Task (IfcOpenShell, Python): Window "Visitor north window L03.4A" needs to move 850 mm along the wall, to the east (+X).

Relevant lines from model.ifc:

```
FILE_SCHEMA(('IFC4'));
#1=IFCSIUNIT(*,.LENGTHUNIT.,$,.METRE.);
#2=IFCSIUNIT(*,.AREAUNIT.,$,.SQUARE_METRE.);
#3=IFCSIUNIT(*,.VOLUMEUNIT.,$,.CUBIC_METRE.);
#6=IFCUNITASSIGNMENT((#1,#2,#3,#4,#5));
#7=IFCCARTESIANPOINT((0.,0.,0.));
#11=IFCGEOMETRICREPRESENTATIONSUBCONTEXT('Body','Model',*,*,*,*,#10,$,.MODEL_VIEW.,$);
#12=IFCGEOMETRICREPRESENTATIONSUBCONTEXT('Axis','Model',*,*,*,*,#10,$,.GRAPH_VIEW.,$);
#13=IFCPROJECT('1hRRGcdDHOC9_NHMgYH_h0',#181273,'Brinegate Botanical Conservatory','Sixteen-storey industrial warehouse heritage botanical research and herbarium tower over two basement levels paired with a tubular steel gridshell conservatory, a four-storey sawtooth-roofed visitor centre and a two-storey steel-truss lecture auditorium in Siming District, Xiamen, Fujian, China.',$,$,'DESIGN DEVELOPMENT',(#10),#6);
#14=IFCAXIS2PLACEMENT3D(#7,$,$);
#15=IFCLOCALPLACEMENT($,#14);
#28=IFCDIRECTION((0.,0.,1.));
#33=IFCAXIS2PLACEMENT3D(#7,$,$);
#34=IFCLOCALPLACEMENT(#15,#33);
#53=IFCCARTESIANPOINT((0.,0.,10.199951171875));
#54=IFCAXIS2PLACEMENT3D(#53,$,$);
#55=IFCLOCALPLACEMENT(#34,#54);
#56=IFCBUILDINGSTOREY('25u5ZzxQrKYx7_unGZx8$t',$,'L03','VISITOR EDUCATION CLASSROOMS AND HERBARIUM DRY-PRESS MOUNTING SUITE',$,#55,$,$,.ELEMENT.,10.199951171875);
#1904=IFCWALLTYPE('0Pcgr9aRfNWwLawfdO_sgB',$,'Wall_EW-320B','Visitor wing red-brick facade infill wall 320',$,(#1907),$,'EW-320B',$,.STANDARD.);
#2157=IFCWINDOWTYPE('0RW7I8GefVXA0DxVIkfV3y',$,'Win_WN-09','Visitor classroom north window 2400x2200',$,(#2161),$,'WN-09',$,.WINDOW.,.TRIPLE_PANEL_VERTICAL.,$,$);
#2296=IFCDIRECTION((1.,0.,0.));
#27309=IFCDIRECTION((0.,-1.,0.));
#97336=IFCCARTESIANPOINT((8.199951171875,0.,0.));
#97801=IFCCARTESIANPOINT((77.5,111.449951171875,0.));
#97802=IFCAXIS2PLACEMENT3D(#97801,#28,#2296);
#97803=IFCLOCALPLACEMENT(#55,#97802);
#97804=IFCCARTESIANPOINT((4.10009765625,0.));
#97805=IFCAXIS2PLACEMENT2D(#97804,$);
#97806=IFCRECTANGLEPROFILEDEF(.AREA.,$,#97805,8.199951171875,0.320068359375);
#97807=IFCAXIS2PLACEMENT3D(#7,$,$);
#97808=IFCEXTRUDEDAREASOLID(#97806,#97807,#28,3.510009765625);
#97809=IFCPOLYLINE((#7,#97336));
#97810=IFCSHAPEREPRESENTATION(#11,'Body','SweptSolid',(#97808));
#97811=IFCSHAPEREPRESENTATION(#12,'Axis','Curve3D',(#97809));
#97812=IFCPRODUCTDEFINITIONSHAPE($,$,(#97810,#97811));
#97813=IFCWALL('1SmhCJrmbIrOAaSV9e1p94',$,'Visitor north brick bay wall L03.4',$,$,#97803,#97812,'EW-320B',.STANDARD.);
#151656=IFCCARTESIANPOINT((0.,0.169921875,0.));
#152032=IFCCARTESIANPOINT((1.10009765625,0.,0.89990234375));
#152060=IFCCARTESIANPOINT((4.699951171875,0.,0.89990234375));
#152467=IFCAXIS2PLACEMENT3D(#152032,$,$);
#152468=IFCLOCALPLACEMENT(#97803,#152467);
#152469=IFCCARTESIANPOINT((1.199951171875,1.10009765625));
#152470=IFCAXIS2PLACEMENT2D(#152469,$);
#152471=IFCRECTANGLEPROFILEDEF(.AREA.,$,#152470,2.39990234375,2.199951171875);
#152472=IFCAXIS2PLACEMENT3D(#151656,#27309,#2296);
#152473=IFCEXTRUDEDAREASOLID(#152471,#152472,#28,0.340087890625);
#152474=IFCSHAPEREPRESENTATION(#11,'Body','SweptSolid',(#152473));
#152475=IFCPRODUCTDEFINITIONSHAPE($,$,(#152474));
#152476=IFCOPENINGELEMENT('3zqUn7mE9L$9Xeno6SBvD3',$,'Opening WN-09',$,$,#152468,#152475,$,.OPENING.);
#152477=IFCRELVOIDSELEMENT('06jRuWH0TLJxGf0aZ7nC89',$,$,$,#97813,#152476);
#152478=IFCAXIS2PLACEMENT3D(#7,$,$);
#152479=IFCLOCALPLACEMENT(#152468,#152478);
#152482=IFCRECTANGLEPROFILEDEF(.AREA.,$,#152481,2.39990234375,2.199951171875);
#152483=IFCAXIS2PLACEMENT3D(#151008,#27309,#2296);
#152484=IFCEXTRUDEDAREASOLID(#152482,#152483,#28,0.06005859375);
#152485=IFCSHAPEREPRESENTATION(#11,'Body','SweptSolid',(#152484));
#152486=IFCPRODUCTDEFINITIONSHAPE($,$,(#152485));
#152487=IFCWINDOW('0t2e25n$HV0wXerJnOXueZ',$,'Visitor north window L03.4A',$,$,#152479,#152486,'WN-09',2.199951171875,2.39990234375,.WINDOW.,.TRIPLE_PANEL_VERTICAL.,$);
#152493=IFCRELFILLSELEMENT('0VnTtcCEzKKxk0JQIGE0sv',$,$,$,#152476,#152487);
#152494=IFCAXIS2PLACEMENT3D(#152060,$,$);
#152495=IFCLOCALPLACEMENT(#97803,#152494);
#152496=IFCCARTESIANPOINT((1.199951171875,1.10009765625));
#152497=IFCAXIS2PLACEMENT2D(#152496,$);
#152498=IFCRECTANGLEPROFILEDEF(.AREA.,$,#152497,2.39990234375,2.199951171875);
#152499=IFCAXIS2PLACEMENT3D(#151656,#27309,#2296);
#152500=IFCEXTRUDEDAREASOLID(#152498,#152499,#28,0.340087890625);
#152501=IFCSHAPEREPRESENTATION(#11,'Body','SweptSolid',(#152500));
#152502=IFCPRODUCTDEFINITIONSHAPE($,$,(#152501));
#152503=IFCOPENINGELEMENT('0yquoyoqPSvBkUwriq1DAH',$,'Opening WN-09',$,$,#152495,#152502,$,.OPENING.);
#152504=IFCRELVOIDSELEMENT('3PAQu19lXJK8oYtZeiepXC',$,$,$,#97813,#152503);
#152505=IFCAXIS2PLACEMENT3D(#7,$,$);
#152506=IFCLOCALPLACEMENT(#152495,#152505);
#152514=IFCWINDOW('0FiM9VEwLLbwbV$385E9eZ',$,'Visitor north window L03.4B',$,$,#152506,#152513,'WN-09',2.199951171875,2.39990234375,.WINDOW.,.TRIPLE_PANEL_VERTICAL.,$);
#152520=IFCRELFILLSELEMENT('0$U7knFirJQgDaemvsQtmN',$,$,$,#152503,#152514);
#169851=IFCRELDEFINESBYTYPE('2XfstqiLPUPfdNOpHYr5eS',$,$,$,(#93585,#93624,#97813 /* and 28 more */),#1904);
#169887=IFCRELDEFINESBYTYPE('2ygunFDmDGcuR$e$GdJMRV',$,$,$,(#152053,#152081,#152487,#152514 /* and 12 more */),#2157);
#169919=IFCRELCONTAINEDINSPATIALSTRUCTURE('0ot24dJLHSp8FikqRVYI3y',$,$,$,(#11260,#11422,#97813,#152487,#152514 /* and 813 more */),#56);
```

```python
import ifcopenshell
import ifcopenshell.api.geometry
import ifcopenshell.util.placement
import ifcopenshell.util.unit

model = ifcopenshell.open("model.ifc")
unit_scale = ifcopenshell.util.unit.calculate_unit_scale(model)

window = model.by_guid("0t2e25n$HV0wXerJnOXueZ")
opening = window.FillsVoids[0].RelatingOpeningElement
wall = opening.VoidsElements[0].RelatingBuildingElement

wall_matrix = ifcopenshell.util.placement.get_local_placement(wall.ObjectPlacement)
shift = wall_matrix[:3, 0] * 0.85 / unit_scale
before = ifcopenshell.util.placement.get_local_placement(window.ObjectPlacement)[:3, 3].copy()

# The window is placed relative to its opening, so it follows when the opening moves.
matrix = ifcopenshell.util.placement.get_local_placement(opening.ObjectPlacement)
matrix[:3, 3] += shift
ifcopenshell.api.geometry.edit_object_placement(
    model, product=opening, matrix=matrix, is_si=False, should_transform_children=True
)

after = ifcopenshell.util.placement.get_local_placement(window.ObjectPlacement)[:3, 3]
print("window moved by", (after - before).round(3) + 0.0)

model.write("model_edited.ifc")
```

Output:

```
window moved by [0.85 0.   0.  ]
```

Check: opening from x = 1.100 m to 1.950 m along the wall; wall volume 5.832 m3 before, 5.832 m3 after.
